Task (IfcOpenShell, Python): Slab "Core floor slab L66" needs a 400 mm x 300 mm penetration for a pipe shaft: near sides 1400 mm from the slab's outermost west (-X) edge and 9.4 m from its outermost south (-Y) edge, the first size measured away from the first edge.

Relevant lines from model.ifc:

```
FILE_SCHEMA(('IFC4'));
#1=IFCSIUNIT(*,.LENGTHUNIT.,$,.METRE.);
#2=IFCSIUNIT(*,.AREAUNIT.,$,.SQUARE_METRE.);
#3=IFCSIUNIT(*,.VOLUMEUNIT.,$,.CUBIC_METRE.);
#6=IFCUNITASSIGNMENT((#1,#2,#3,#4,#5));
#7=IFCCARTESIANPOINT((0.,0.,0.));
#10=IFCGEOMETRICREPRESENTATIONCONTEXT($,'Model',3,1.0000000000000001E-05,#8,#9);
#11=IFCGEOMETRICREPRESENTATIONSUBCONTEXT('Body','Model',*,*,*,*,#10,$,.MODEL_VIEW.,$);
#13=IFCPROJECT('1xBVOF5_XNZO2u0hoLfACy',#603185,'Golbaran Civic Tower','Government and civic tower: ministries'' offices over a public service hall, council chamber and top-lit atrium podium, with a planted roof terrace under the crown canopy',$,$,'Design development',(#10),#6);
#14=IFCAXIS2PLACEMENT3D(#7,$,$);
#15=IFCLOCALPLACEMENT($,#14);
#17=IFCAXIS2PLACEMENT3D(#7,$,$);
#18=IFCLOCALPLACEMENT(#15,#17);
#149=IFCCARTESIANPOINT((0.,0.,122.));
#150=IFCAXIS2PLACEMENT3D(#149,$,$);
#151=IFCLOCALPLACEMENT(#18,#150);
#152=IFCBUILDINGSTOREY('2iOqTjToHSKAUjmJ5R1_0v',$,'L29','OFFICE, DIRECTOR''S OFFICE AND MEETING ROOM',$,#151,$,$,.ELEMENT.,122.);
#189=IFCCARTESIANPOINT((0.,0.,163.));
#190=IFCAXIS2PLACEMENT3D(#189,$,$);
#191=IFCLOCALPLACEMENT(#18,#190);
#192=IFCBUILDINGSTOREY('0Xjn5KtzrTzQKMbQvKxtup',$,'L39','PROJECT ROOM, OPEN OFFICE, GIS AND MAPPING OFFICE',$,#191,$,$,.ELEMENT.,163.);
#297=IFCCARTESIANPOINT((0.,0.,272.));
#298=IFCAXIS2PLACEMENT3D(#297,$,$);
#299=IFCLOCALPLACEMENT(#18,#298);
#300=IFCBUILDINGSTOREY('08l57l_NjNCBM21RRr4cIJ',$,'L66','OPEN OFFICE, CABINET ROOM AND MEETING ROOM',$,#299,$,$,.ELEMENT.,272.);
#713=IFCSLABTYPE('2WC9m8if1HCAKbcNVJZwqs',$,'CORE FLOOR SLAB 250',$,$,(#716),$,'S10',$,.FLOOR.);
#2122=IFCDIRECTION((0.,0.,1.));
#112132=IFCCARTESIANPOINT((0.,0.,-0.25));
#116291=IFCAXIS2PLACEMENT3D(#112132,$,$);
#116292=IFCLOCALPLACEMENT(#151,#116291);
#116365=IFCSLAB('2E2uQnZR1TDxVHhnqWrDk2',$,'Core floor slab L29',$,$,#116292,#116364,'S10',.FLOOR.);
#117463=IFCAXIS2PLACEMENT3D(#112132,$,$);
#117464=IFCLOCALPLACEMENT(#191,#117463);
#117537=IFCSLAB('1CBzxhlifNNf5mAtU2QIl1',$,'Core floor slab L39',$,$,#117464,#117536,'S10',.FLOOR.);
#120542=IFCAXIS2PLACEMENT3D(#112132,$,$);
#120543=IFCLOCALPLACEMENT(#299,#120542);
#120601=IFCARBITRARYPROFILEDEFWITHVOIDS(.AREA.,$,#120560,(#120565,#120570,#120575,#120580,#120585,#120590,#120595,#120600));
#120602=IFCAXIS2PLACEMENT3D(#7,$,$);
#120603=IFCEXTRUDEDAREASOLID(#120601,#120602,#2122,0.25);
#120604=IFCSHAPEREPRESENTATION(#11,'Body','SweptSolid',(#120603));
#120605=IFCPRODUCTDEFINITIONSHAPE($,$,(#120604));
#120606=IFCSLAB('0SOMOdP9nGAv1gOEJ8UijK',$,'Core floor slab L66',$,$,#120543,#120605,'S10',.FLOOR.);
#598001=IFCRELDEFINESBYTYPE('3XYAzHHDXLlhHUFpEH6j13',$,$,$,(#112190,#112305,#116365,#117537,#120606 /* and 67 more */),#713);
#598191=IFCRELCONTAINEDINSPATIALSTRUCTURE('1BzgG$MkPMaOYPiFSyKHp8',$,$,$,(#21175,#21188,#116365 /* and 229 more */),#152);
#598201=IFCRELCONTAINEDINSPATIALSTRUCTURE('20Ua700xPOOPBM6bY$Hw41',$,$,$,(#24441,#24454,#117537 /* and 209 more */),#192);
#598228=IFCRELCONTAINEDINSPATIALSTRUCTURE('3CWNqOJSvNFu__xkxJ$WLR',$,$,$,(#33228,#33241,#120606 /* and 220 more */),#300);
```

```python
import numpy as np
import ifcopenshell
import ifcopenshell.api.feature
import ifcopenshell.api.geometry
import ifcopenshell.api.root
import ifcopenshell.geom
import ifcopenshell.util.placement
import ifcopenshell.util.representation
import ifcopenshell.util.shape
import ifcopenshell.util.unit

model = ifcopenshell.open("model.ifc")
unit_scale = ifcopenshell.util.unit.calculate_unit_scale(model)
settings = ifcopenshell.geom.settings()


def volume(element):
    """Net volume in cubic metres, openings subtracted."""
    shape = ifcopenshell.geom.create_shape(settings, element)
    return ifcopenshell.util.shape.get_volume(shape.geometry)


slab = model.by_guid("0SOMOdP9nGAv1gOEJ8UijK")
before = volume(slab)

# Extent in the slab's own axes, in metres. The edges named are its -X and -Y sides.
slab_shape = ifcopenshell.geom.create_shape(settings, slab)
vertices = ifcopenshell.util.shape.get_vertices(slab_shape.geometry)
x_min, y_min, bottom = vertices.min(axis=0)
top = vertices[:, 2].max()

opening = ifcopenshell.api.root.create_entity(model, ifc_class="IfcOpeningElement", name="Pipe shaft opening", predefined_type="OPENING")
context = ifcopenshell.util.representation.get_context(model, "Model", "Body", "MODEL_VIEW")
width, depth = 0.4, 0.3
outline = [(0.0, 0.0), (width, 0.0), (width, depth), (0.0, depth), (0.0, 0.0)]
# Overshoot both faces by 50 mm so the cut is clean.
shape = ifcopenshell.api.geometry.add_slab_representation(
    model, context=context, depth=top - bottom + 0.1, polyline=outline
)
ifcopenshell.api.geometry.assign_representation(model, product=opening, representation=shape)

matrix = ifcopenshell.util.placement.get_local_placement(slab.ObjectPlacement)
matrix[:, 3] = matrix @ np.append(np.array([x_min + 1.4, y_min + 9.4, bottom - 0.05]) / unit_scale, 1.0)
ifcopenshell.api.geometry.edit_object_placement(model, product=opening, matrix=matrix, is_si=False)
ifcopenshell.api.feature.add_feature(model, feature=opening, element=slab)

after = volume(slab)

print(f"slab volume {before:.3f} -> {after:.3f} m3")

model.write("model_edited.ifc")
```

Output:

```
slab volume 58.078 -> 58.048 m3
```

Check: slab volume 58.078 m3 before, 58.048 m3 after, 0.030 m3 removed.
